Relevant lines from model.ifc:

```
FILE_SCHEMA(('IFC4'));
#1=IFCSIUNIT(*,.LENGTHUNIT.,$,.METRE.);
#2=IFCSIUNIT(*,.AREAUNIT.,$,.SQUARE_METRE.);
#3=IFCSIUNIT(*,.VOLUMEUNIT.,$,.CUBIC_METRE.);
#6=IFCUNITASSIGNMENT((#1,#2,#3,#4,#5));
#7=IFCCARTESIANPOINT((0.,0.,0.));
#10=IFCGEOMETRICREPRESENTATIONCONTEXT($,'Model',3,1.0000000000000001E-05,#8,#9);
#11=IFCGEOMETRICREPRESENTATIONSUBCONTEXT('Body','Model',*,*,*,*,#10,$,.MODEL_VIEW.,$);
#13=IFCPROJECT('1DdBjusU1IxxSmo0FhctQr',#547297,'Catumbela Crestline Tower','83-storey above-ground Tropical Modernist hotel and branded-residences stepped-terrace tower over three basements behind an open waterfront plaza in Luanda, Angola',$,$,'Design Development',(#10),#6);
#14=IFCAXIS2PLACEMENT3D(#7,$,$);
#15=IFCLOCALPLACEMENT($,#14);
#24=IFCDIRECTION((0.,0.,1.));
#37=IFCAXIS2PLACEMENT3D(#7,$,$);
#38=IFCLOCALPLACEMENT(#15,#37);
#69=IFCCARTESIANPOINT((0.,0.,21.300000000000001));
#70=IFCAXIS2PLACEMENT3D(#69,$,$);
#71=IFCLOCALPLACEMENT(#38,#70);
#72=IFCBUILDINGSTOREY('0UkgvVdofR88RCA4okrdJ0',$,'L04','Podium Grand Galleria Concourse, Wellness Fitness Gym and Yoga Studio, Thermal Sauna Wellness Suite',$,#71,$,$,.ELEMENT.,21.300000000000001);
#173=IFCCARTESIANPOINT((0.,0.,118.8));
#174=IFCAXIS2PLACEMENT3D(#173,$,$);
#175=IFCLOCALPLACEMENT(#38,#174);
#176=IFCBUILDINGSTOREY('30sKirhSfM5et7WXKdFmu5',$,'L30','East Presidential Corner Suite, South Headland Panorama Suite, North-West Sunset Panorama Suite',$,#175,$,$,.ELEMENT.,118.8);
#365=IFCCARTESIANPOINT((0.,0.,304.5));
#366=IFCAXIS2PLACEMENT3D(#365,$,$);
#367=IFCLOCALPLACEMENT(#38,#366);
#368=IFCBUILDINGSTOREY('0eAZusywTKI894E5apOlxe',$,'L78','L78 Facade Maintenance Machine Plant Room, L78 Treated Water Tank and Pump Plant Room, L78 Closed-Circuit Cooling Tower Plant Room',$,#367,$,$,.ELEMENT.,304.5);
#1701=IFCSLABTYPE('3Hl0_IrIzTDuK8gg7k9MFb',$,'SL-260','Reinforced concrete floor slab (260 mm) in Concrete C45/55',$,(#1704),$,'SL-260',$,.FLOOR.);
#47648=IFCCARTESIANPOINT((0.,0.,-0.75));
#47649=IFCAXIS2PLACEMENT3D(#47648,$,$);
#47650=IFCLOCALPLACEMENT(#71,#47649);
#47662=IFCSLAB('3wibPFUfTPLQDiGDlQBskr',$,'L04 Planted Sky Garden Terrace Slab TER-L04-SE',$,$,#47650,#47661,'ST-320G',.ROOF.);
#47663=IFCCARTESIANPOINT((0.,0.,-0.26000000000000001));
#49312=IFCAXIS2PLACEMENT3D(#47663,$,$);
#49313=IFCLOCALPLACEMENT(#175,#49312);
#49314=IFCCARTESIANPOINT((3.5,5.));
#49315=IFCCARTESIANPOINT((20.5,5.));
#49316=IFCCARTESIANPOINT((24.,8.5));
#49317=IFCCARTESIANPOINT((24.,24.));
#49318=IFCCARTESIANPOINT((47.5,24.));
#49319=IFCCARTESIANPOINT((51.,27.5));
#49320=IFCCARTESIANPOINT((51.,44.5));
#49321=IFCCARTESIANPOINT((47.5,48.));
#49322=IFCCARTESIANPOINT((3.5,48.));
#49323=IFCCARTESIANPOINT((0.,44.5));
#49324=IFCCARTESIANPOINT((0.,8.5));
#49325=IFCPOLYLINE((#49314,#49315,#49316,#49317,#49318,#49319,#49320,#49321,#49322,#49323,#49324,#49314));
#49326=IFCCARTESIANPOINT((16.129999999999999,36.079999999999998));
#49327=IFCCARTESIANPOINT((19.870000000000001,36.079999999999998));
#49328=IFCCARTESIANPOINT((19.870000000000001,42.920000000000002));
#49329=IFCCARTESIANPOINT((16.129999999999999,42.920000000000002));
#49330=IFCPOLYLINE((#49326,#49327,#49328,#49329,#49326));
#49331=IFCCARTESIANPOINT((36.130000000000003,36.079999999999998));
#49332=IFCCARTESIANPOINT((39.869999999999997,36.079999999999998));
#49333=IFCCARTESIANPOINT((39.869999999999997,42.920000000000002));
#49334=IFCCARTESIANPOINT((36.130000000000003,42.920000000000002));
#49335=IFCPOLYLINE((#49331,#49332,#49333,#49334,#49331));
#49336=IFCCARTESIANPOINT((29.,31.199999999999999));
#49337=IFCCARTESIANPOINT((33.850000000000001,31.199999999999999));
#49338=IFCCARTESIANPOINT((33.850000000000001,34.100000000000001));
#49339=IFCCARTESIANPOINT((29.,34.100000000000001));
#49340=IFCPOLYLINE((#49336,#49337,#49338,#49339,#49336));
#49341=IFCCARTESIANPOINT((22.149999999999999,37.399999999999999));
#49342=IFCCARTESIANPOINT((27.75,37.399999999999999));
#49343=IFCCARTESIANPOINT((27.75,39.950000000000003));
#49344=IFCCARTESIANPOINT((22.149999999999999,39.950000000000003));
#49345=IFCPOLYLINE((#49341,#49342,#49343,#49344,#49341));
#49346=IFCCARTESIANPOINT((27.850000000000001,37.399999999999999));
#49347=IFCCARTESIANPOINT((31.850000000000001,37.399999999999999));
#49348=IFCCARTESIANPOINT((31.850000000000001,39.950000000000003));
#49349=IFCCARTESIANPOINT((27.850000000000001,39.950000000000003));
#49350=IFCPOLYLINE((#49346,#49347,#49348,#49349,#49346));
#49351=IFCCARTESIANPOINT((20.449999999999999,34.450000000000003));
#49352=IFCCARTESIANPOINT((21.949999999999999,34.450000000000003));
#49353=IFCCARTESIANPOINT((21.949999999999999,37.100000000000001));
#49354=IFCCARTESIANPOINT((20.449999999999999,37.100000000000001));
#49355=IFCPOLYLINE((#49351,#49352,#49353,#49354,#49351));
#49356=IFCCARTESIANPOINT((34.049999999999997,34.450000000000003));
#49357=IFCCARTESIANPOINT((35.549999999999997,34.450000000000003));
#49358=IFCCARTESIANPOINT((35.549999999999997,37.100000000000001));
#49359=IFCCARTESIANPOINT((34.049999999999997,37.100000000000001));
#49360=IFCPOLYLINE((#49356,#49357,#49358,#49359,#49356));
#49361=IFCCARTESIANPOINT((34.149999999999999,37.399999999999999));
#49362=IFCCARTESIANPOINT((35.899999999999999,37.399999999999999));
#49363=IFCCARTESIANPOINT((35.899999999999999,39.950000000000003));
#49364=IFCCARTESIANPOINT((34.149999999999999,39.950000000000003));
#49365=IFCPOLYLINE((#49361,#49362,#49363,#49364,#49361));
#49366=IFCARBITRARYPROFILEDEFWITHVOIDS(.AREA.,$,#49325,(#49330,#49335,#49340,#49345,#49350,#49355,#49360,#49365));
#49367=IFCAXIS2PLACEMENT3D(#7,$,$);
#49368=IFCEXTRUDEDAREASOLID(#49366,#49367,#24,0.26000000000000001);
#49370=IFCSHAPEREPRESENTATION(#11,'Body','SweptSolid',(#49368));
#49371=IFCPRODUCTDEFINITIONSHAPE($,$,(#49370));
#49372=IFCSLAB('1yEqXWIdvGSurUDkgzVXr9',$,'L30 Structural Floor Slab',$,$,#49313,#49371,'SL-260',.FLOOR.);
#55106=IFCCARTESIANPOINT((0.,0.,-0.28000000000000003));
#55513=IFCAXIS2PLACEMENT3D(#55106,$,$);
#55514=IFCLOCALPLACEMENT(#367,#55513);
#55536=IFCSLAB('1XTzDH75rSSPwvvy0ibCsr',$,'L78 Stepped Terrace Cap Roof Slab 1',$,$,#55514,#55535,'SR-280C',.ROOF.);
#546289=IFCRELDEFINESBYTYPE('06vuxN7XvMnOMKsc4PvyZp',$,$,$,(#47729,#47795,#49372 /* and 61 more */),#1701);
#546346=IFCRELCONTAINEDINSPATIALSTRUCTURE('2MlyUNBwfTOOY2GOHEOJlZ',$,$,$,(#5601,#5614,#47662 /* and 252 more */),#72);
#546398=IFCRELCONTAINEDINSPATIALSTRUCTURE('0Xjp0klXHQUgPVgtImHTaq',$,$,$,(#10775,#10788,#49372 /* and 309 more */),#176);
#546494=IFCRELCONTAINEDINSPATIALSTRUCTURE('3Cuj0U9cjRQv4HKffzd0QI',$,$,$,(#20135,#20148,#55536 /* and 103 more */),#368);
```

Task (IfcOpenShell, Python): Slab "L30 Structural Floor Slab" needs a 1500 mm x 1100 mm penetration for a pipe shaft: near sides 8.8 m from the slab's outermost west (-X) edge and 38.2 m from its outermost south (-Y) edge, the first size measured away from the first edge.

```python
import numpy as np
import ifcopenshell
import ifcopenshell.api.feature
import ifcopenshell.api.geometry
import ifcopenshell.api.root
import ifcopenshell.geom
import ifcopenshell.util.placement
import ifcopenshell.util.representation
import ifcopenshell.util.shape
import ifcopenshell.util.unit

model = ifcopenshell.open("model.ifc")
unit_scale = ifcopenshell.util.unit.calculate_unit_scale(model)
settings = ifcopenshell.geom.settings()


def volume(element):
    """Net volume in cubic metres, openings subtracted."""
    shape = ifcopenshell.geom.create_shape(settings, element)
    return ifcopenshell.util.shape.get_volume(shape.geometry)


slab = model.by_guid("1yEqXWIdvGSurUDkgzVXr9")
before = volume(slab)

# Extent in the slab's own axes, in metres. The edges named are its -X and -Y sides.
slab_shape = ifcopenshell.geom.create_shape(settings, slab)
vertices = ifcopenshell.util.shape.get_vertices(slab_shape.geometry)
x_min, y_min, bottom = vertices.min(axis=0)
top = vertices[:, 2].max()

opening = ifcopenshell.api.root.create_entity(model, ifc_class="IfcOpeningElement", name="Pipe shaft opening", predefined_type="OPENING")
context = ifcopenshell.util.representation.get_context(model, "Model", "Body", "MODEL_VIEW")
width, depth = 1.5, 1.1
outline = [(0.0, 0.0), (width, 0.0), (width, depth), (0.0, depth), (0.0, 0.0)]
# Overshoot both faces by 50 mm so the cut is clean.
shape = ifcopenshell.api.geometry.add_slab_representation(
    model, context=context, depth=top - bottom + 0.1, polyline=outline
)
ifcopenshell.api.geometry.assign_representation(model, product=opening, representation=shape)

matrix = ifcopenshell.util.placement.get_local_placement(slab.ObjectPlacement)
matrix[:, 3] = matrix @ np.append(np.array([x_min + 8.8, y_min + 38.2, bottom - 0.05]) / unit_scale, 1.0)
ifcopenshell.api.geometry.edit_object_placement(model, product=opening, matrix=matrix, is_si=False)
ifcopenshell.api.feature.add_feature(model, feature=opening, element=slab)

after = volume(slab)

print(f"slab volume {before:.3f} -> {after:.3f} m3")

model.write("model_edited.ifc")
```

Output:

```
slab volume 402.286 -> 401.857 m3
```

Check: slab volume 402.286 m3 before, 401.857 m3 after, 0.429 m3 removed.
